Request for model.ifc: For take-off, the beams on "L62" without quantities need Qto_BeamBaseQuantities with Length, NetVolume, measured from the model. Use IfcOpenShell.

First a look at what the model holds.

```python
import ifcopenshell
import ifcopenshell.util.element
import ifcopenshell.util.unit

model = ifcopenshell.open("model.ifc")
print(model.schema)
for unit_type in ("LENGTHUNIT", "AREAUNIT", "VOLUMEUNIT"):
    print(unit_type, ifcopenshell.util.unit.calculate_unit_scale(model, unit_type))
storey = next(s for s in model.by_type("IfcBuildingStorey") if s.Name == "L62")
beams = [e for e in ifcopenshell.util.element.get_decomposition(storey) if e.is_a("IfcBeam")]
for e in sorted(beams, key=lambda e: e.id()):
    print(e.id(), e.is_a(), e.Name, list(ifcopenshell.util.element.get_psets(e, qtos_only=True)), sep=" | ")
```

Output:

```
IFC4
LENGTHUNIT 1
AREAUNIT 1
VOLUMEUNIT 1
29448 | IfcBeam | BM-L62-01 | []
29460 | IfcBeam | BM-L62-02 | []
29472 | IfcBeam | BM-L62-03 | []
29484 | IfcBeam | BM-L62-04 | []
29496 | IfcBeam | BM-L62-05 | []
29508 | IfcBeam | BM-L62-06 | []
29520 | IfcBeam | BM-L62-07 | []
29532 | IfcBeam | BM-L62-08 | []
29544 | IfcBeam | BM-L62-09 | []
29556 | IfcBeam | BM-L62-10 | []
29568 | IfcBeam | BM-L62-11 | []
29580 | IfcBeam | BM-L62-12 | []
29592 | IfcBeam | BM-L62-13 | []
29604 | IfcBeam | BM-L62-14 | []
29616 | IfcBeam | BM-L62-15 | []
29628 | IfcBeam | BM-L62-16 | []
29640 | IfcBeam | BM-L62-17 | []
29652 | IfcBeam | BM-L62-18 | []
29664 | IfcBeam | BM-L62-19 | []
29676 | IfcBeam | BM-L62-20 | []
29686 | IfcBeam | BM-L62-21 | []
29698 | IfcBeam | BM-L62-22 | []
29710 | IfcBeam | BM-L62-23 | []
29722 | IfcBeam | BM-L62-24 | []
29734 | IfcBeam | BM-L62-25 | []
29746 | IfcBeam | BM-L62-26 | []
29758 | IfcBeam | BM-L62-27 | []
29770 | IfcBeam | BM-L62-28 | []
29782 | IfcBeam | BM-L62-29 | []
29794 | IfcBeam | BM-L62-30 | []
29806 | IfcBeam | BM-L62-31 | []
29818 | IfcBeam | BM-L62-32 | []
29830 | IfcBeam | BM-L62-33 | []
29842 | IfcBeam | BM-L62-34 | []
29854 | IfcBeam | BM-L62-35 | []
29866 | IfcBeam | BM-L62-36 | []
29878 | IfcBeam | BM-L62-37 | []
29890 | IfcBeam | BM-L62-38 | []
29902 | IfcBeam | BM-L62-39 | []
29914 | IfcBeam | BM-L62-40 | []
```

```python
import ifcopenshell
import ifcopenshell.api.pset
import ifcopenshell.geom
import ifcopenshell.util.element
import ifcopenshell.util.shape
import ifcopenshell.util.unit

model = ifcopenshell.open("model.ifc")
unit_scale = ifcopenshell.util.unit.calculate_unit_scale(model)
volume_scale = ifcopenshell.util.unit.calculate_unit_scale(model, "VOLUMEUNIT")
settings = ifcopenshell.geom.settings()

storey = next(s for s in model.by_type("IfcBuildingStorey") if s.Name == "L62")
beams = [e for e in ifcopenshell.util.element.get_decomposition(storey) if e.is_a("IfcBeam")]

for e in sorted(beams, key=lambda e: e.id()):
    if ifcopenshell.util.element.get_psets(e, qtos_only=True, should_inherit=False):
        continue
    # Geometry comes back in metres, in the element's own axes.
    shape = ifcopenshell.geom.create_shape(settings, e)
    values = {
        "Length": ifcopenshell.util.shape.get_max_xyz(shape.geometry) / unit_scale,
        "NetVolume": ifcopenshell.util.shape.get_volume(shape.geometry) / volume_scale,
    }
    qto = ifcopenshell.api.pset.add_qto(model, product=e, name="Qto_BeamBaseQuantities")
    ifcopenshell.api.pset.edit_qto(model, qto=qto, properties=values)
    print(e.id(), {k: round(v, 3) for k, v in values.items()})

model.write("model-out.ifc")
```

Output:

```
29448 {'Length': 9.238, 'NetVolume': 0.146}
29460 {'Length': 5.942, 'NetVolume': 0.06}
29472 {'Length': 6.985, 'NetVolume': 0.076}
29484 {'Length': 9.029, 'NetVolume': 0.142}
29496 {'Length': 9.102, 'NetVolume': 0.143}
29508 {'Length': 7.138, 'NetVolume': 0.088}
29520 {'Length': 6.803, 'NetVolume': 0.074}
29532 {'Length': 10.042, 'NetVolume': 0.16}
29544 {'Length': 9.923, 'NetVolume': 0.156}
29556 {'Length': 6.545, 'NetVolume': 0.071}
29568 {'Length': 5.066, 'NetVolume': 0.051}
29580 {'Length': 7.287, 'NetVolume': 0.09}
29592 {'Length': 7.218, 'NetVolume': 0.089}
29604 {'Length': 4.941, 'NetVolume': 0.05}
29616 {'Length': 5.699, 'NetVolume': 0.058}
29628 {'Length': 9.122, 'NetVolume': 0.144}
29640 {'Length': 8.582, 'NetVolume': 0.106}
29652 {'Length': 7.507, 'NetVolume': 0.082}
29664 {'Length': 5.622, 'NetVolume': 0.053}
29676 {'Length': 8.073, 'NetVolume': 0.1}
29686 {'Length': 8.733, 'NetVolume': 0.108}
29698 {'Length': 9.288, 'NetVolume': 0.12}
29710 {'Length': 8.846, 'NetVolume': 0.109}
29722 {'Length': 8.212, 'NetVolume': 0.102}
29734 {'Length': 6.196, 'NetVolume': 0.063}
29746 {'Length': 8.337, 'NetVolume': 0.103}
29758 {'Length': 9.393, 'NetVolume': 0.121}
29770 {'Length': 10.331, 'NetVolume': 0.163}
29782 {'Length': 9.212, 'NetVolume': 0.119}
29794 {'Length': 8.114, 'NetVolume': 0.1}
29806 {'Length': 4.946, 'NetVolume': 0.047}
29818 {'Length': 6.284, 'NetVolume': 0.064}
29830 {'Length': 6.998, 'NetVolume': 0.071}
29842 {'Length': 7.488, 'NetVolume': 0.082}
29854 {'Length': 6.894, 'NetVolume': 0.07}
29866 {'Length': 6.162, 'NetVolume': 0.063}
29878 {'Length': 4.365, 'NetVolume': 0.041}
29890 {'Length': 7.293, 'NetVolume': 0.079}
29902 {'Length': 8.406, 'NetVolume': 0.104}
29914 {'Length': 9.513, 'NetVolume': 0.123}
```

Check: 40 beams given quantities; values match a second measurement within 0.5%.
